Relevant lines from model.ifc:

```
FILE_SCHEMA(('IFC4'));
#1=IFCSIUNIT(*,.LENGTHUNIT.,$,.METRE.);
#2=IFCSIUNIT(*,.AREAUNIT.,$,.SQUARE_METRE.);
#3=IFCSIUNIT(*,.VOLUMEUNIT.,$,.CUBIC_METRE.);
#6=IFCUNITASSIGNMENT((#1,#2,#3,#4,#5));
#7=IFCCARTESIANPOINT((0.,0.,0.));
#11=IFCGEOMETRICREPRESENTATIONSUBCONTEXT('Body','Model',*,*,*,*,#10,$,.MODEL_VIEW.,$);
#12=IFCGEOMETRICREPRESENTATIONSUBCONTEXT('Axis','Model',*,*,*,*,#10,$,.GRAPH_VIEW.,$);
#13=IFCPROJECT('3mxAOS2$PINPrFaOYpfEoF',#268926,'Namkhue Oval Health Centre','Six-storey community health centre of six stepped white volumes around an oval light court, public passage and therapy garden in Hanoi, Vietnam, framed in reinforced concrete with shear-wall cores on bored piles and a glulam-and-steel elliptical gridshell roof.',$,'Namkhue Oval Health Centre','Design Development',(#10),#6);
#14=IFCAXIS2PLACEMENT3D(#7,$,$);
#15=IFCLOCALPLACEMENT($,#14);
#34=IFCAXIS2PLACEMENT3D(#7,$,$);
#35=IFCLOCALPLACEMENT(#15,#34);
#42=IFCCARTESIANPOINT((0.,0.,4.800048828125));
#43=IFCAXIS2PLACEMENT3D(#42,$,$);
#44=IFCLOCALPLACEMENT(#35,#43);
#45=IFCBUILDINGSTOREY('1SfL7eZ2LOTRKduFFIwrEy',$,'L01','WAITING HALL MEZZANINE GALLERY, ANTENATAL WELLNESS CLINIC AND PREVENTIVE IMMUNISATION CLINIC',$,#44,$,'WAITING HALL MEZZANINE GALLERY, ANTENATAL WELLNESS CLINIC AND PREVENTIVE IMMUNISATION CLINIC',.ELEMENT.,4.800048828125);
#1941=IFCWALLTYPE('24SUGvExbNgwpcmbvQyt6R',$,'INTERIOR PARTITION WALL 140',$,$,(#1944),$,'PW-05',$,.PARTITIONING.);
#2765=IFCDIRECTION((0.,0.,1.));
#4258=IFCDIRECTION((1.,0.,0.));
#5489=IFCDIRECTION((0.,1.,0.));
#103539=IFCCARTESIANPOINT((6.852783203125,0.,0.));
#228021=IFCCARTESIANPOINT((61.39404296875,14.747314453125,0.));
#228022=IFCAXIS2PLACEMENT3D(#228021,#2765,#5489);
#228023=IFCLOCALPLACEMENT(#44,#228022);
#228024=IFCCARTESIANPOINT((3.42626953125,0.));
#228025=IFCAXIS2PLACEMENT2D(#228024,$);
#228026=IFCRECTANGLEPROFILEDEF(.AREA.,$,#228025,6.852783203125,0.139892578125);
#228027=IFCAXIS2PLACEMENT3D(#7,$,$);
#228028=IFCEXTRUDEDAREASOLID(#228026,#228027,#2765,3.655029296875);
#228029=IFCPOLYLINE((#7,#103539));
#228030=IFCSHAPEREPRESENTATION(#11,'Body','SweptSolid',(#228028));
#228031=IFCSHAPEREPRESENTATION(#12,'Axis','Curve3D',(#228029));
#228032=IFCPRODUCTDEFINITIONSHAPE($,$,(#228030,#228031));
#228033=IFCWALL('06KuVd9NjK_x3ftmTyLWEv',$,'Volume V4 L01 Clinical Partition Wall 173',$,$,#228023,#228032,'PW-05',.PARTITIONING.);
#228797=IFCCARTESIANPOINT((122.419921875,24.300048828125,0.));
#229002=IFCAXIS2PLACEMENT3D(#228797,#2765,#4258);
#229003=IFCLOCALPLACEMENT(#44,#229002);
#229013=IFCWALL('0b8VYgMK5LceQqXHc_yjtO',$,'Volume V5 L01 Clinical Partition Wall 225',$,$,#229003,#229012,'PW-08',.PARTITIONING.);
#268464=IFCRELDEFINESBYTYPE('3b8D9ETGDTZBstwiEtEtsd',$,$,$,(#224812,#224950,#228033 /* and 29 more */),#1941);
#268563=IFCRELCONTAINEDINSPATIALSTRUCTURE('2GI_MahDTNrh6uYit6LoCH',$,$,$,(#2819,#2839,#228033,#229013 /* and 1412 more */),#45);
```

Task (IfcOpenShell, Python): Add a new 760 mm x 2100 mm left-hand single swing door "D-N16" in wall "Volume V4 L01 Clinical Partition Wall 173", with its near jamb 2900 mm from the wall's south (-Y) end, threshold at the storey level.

```python
import numpy as np
import ifcopenshell
import ifcopenshell.api.feature
import ifcopenshell.api.geometry
import ifcopenshell.api.root
import ifcopenshell.api.spatial
import ifcopenshell.geom
import ifcopenshell.util.element
import ifcopenshell.util.placement
import ifcopenshell.util.representation
import ifcopenshell.util.shape
import ifcopenshell.util.unit

model = ifcopenshell.open("model.ifc")
unit_scale = ifcopenshell.util.unit.calculate_unit_scale(model)
settings = ifcopenshell.geom.settings()


def volume(element):
    """Net volume in cubic metres, openings subtracted."""
    shape = ifcopenshell.geom.create_shape(settings, element)
    return ifcopenshell.util.shape.get_volume(shape.geometry)


wall = model.by_id(228033)
storey = ifcopenshell.util.element.get_container(wall, ifc_class="IfcBuildingStorey")
context = ifcopenshell.util.representation.get_context(model, "Model", "Body", "MODEL_VIEW")
before = volume(wall)

width, height, from_end, sill = 0.76, 2.1, 2.9, 0.0  # metres

# The wall runs along its own X axis, and the end named is its -X end.
wall_shape = ifcopenshell.geom.create_shape(settings, wall)
x, y, z = ifcopenshell.util.shape.get_vertices(wall_shape.geometry).T
start = x.min() + from_end
face, thickness = float(y.min()), float(y.max() - y.min())
wall_matrix = ifcopenshell.util.placement.get_local_placement(wall.ObjectPlacement)
level = ifcopenshell.util.placement.get_local_placement(storey.ObjectPlacement)[2, 3]


def in_wall(x, y):
    """Placement at x, y metres in the wall's axes, at sill height."""
    matrix = wall_matrix.copy()
    matrix[:, 3] = wall_matrix @ np.array([x / unit_scale, y / unit_scale, 0.0, 1.0])
    matrix[2, 3] = level + sill / unit_scale
    return matrix


# Opening: a box that overshoots both wall faces by 50 mm.
opening = ifcopenshell.api.root.create_entity(model, ifc_class="IfcOpeningElement", predefined_type="OPENING")
box = ifcopenshell.api.geometry.add_wall_representation(
    model, context=context, length=width, height=height, thickness=thickness + 0.1
)
ifcopenshell.api.geometry.assign_representation(model, product=opening, representation=box)
ifcopenshell.api.geometry.edit_object_placement(model, product=opening, matrix=in_wall(start, face - 0.05), is_si=False)
ifcopenshell.api.feature.add_feature(model, feature=opening, element=wall)

door = ifcopenshell.api.root.create_entity(model, ifc_class="IfcDoor", name="D-N16", predefined_type="DOOR")
door.OverallWidth, door.OverallHeight = width / unit_scale, height / unit_scale
door.OperationType = "SINGLE_SWING_LEFT"
body = ifcopenshell.api.geometry.add_door_representation(
    model,
    context=context,
    overall_width=door.OverallWidth,
    overall_height=door.OverallHeight,
    operation_type="SINGLE_SWING_LEFT",
    lining_properties={"LiningDepth": thickness / unit_scale, "ThresholdDepth": thickness / unit_scale},
)
ifcopenshell.api.geometry.assign_representation(model, product=door, representation=body)
ifcopenshell.api.spatial.assign_container(model, products=[door], relating_structure=storey)
ifcopenshell.api.feature.add_filling(model, opening=opening, element=door)

# The lining spans the wall, so the door starts at the wall face.
ifcopenshell.api.geometry.edit_object_placement(model, product=door, matrix=in_wall(start, face), is_si=False)

after = volume(wall)

print(f"wall volume {before:.3f} -> {after:.3f} m3")

model.write("model_edited.ifc")
```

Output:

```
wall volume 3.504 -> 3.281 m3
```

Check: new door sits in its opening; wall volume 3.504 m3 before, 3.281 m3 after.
